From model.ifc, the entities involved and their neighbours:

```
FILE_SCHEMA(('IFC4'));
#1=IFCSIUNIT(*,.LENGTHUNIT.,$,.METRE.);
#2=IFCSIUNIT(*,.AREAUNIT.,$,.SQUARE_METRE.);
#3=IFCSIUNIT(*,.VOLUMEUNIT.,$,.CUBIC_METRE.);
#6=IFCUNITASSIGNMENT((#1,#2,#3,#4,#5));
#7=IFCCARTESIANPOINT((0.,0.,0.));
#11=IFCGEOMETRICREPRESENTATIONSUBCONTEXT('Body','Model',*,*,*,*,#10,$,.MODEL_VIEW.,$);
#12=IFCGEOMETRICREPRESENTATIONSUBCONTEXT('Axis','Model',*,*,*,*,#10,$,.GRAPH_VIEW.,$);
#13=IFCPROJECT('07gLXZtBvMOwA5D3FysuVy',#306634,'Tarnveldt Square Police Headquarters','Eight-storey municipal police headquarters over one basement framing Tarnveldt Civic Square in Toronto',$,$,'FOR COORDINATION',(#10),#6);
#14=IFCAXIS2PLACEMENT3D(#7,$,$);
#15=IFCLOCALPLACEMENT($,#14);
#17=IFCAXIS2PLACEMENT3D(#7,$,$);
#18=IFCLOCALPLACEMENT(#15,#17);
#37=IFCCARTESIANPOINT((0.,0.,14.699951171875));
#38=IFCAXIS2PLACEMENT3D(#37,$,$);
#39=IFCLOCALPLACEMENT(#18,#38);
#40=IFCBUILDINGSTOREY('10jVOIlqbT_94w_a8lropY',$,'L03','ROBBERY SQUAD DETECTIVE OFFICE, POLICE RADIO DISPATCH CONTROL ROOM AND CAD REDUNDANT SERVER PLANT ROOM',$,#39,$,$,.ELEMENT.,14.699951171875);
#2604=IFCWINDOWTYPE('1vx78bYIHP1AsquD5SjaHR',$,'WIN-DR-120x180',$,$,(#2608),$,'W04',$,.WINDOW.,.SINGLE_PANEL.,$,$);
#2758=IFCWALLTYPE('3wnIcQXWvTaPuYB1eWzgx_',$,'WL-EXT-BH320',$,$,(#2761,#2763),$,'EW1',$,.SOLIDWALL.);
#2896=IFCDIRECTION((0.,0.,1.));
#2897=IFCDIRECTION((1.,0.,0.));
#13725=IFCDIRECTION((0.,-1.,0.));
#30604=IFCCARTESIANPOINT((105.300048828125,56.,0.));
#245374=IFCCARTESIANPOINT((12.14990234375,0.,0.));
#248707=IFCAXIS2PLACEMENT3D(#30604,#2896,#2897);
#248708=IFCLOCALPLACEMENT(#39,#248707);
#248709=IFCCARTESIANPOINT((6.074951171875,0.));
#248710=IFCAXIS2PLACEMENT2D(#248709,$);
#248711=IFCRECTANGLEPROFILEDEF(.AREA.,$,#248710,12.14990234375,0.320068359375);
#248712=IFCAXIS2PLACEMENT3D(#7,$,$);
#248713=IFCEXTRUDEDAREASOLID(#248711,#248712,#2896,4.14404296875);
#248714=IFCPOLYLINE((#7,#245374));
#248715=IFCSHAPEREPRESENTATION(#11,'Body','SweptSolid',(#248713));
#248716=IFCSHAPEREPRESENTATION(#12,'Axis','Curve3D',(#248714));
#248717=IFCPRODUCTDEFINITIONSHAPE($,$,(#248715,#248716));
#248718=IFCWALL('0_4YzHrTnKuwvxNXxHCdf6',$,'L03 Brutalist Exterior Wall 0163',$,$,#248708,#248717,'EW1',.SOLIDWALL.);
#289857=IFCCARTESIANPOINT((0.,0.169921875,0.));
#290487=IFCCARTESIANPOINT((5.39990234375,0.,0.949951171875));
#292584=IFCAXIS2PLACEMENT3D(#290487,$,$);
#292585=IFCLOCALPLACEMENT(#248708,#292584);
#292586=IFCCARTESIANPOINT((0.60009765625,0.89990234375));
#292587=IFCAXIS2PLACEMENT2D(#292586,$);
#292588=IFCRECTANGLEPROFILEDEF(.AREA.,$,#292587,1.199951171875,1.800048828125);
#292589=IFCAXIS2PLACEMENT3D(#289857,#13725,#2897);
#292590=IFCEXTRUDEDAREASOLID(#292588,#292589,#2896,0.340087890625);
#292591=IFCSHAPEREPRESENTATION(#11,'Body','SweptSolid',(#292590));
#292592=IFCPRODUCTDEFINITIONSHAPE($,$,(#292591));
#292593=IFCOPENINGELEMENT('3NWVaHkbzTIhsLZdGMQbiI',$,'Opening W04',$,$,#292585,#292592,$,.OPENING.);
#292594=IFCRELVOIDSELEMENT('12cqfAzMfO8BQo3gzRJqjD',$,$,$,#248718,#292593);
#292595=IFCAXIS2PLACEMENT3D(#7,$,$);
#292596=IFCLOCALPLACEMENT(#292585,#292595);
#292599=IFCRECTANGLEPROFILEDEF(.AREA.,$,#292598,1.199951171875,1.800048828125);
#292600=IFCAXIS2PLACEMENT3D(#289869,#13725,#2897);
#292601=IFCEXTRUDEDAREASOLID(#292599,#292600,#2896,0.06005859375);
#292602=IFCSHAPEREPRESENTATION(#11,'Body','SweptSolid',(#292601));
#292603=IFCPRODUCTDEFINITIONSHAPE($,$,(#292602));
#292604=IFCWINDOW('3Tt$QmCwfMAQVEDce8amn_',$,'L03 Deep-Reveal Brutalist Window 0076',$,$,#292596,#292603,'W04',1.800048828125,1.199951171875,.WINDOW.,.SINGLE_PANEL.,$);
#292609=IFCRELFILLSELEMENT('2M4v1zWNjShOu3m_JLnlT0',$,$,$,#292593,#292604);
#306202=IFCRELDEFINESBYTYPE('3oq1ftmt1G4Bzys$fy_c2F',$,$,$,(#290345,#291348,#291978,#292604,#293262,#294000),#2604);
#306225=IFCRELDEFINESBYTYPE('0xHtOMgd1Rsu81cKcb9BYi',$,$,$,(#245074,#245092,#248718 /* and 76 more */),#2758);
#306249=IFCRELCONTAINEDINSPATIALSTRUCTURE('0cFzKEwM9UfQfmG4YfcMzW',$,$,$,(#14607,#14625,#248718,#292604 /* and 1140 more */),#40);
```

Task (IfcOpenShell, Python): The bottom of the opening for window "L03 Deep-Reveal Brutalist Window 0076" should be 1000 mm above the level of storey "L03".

```python
import numpy as np
import ifcopenshell
import ifcopenshell.api.geometry
import ifcopenshell.geom
import ifcopenshell.util.element
import ifcopenshell.util.placement
import ifcopenshell.util.shape
import ifcopenshell.util.unit

model = ifcopenshell.open("model.ifc")
unit_scale = ifcopenshell.util.unit.calculate_unit_scale(model)

window = model.by_guid("3Tt$QmCwfMAQVEDce8amn_")
opening = window.FillsVoids[0].RelatingOpeningElement
storey = ifcopenshell.util.element.get_container(window, ifc_class="IfcBuildingStorey")
level = ifcopenshell.util.placement.get_local_placement(storey.ObjectPlacement)[2, 3]

# The opening's origin need not be at the sill, so measure its lowest point.
shape = ifcopenshell.geom.create_shape(ifcopenshell.geom.settings(), opening)
bottom = ifcopenshell.util.shape.get_shape_bottom_elevation(shape, shape.geometry) / unit_scale
dz = level + 1 / unit_scale - bottom

shift = np.array([0.0, 0.0, dz])
# The window is placed relative to its opening, so it follows when the opening moves.
matrix = ifcopenshell.util.placement.get_local_placement(opening.ObjectPlacement)
matrix[:3, 3] += shift
ifcopenshell.api.geometry.edit_object_placement(
    model, product=opening, matrix=matrix, is_si=False, should_transform_children=True
)

print(f"moved by {dz * unit_scale:+.3f} m")

model.write("model_edited.ifc")
```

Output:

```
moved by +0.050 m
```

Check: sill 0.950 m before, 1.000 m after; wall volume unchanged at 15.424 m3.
